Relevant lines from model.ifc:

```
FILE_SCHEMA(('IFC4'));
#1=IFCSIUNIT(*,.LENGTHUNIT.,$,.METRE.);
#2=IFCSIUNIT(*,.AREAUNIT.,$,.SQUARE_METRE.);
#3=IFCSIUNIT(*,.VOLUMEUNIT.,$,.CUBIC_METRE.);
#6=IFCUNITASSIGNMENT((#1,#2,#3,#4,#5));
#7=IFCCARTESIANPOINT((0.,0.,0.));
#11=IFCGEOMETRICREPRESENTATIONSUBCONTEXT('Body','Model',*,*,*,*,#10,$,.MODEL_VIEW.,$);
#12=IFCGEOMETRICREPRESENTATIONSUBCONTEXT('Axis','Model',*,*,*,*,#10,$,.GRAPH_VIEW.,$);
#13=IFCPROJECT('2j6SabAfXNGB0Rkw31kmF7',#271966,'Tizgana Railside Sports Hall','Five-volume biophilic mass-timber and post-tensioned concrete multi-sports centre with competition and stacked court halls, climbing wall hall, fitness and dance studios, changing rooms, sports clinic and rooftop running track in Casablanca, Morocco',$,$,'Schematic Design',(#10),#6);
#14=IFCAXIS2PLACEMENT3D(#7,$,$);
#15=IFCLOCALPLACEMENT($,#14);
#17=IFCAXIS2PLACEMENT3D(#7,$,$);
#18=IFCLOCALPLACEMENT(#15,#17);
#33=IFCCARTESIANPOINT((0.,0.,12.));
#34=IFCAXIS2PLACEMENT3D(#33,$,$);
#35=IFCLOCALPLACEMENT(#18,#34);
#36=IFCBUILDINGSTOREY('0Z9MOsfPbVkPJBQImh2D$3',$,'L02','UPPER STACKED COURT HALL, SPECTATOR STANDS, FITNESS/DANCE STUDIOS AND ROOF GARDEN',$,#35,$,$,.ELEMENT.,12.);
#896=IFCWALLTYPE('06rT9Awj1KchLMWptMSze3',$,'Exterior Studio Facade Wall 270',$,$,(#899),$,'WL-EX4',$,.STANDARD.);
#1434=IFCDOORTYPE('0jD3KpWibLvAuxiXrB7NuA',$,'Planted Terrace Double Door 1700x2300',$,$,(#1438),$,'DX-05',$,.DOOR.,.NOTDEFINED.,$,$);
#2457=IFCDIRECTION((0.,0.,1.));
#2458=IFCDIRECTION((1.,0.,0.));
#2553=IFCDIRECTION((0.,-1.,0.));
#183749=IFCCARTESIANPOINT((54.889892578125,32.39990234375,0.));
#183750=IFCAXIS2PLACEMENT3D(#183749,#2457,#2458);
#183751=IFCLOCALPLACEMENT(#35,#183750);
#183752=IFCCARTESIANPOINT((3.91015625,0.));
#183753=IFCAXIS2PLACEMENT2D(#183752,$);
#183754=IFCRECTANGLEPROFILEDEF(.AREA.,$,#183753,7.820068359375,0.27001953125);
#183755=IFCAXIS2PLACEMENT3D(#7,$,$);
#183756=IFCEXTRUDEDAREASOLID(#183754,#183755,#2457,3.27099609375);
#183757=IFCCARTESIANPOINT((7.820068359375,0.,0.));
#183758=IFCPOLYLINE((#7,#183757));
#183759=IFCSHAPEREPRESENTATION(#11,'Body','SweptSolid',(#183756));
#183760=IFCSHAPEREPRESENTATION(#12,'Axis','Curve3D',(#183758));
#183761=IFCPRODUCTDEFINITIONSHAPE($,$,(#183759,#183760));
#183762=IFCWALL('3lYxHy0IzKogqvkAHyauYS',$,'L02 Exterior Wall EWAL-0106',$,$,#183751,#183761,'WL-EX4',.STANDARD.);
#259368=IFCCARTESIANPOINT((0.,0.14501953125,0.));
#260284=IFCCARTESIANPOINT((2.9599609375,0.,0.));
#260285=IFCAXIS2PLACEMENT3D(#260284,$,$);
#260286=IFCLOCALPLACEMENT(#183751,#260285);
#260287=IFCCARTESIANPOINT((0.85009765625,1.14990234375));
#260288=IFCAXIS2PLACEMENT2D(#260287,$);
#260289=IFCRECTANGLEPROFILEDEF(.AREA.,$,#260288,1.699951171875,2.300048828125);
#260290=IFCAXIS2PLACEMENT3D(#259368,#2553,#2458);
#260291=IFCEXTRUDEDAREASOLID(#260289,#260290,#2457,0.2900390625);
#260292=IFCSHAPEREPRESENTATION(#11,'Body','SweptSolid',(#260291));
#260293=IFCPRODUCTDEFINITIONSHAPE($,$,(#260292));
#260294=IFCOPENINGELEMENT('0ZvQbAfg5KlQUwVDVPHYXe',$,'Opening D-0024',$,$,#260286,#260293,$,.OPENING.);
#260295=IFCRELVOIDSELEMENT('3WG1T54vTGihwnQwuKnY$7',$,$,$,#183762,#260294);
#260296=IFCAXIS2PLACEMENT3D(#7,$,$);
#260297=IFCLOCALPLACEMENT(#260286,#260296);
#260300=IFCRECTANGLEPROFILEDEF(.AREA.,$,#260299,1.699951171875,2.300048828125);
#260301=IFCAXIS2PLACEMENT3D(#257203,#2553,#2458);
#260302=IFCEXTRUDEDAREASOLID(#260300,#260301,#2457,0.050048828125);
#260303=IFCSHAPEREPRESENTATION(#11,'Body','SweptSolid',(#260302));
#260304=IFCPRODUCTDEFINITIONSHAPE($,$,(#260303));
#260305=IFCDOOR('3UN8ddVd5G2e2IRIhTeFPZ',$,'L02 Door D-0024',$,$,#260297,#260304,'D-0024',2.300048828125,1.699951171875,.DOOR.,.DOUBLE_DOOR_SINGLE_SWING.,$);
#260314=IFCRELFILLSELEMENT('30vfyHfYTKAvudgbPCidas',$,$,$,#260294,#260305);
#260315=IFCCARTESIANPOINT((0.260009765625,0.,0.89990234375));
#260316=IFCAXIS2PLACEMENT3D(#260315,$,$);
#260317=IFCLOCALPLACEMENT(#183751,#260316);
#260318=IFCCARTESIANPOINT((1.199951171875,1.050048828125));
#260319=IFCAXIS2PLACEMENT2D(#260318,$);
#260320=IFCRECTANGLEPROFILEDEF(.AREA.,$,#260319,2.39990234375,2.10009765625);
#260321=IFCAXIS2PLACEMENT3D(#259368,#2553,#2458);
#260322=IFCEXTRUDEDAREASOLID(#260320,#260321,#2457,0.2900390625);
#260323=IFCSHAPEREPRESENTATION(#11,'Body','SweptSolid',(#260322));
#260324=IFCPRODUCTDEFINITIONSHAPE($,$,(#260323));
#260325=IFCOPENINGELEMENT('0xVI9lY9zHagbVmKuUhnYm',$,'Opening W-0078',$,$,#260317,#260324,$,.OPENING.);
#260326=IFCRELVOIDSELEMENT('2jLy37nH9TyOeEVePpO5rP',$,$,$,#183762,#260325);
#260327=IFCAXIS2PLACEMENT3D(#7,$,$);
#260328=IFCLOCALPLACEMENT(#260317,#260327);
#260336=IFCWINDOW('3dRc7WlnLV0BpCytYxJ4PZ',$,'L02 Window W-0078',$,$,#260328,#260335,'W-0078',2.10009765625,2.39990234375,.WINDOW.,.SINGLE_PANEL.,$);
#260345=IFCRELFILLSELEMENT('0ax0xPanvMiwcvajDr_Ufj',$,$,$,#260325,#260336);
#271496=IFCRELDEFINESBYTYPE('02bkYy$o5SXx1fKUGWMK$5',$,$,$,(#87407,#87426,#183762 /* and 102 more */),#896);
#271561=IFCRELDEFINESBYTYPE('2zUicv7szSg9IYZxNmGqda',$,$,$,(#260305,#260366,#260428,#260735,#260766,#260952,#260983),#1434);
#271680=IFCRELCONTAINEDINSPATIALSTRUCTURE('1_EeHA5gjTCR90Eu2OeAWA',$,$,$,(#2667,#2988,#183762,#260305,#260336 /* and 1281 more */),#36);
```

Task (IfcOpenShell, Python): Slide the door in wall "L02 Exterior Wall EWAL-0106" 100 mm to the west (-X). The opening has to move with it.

```python
import ifcopenshell
import ifcopenshell.api.geometry
import ifcopenshell.util.placement

model = ifcopenshell.open("model.ifc")

door = model.by_guid("3UN8ddVd5G2e2IRIhTeFPZ")
opening = door.FillsVoids[0].RelatingOpeningElement
wall = opening.VoidsElements[0].RelatingBuildingElement

wall_matrix = ifcopenshell.util.placement.get_local_placement(wall.ObjectPlacement)
shift = wall_matrix[:3, 0] * -0.1
before = ifcopenshell.util.placement.get_local_placement(door.ObjectPlacement)[:3, 3].copy()

# The door is placed relative to its opening, so it follows when the opening moves.
matrix = ifcopenshell.util.placement.get_local_placement(opening.ObjectPlacement)
matrix[:3, 3] += shift
ifcopenshell.api.geometry.edit_object_placement(
    model, product=opening, matrix=matrix, is_si=False, should_transform_children=True
)

after = ifcopenshell.util.placement.get_local_placement(door.ObjectPlacement)[:3, 3]
print("door moved by", (after - before).round(3) + 0.0)

model.write("model_rev.ifc")
```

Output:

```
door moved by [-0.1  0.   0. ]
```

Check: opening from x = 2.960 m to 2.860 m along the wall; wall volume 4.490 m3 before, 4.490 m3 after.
